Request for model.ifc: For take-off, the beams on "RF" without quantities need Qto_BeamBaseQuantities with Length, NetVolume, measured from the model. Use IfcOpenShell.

First a look at what the model holds.

```python
import ifcopenshell
import ifcopenshell.util.element
import ifcopenshell.util.unit

model = ifcopenshell.open("model.ifc")
print(model.schema)
for unit_type in ("LENGTHUNIT", "AREAUNIT", "VOLUMEUNIT"):
    print(unit_type, ifcopenshell.util.unit.calculate_unit_scale(model, unit_type))
storey = next(s for s in model.by_type("IfcBuildingStorey") if s.Name == "RF")
beams = [e for e in ifcopenshell.util.element.get_decomposition(storey) if e.is_a("IfcBeam")]
for e in sorted(beams, key=lambda e: e.id()):
    print(e.id(), e.is_a(), e.Name, list(ifcopenshell.util.element.get_psets(e, qtos_only=True)), sep=" | ")
```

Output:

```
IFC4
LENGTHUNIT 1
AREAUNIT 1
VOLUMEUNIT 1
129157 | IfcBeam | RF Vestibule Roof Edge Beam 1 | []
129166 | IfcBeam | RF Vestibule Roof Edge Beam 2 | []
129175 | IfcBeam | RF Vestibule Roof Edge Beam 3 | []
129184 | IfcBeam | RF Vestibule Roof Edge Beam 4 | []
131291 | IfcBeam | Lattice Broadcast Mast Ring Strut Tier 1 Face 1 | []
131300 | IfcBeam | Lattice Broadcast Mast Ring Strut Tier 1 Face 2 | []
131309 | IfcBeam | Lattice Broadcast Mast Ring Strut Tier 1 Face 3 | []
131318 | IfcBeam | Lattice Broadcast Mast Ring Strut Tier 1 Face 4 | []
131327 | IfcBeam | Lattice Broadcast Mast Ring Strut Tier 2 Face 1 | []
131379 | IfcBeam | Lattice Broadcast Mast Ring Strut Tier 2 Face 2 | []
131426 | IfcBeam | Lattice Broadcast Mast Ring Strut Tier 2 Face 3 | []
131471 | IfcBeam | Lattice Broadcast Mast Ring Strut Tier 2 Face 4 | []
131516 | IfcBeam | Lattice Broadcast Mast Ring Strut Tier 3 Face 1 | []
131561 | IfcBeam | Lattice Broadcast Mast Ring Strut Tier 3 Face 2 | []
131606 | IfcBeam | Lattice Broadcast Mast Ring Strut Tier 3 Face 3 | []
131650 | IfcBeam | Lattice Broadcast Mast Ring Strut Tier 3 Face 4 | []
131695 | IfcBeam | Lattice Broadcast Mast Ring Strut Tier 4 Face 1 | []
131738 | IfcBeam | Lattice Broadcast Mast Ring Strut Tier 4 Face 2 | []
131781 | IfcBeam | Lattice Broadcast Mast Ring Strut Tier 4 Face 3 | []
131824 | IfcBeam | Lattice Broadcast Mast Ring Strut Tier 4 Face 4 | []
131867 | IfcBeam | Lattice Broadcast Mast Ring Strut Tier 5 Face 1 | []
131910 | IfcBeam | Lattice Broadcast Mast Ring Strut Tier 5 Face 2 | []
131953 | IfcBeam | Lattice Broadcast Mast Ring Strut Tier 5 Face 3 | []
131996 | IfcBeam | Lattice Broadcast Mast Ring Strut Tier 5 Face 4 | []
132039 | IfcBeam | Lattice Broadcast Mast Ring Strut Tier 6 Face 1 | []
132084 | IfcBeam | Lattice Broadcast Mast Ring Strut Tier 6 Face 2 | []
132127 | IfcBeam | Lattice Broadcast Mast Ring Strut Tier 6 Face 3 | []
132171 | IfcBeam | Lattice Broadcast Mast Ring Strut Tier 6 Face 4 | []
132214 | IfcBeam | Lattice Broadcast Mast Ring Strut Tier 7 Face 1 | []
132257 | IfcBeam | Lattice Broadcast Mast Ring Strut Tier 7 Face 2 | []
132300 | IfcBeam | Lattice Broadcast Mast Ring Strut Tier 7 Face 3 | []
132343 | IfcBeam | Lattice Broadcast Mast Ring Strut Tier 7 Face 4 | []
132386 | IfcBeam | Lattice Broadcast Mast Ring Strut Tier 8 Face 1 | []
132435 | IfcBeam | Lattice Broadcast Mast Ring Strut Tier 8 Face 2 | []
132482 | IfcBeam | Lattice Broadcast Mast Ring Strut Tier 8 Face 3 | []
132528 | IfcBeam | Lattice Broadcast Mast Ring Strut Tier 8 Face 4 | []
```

```python
import ifcopenshell
import ifcopenshell.api.pset
import ifcopenshell.geom
import ifcopenshell.util.element
import ifcopenshell.util.shape
import ifcopenshell.util.unit

model = ifcopenshell.open("model.ifc")
unit_scale = ifcopenshell.util.unit.calculate_unit_scale(model)
volume_scale = ifcopenshell.util.unit.calculate_unit_scale(model, "VOLUMEUNIT")
settings = ifcopenshell.geom.settings()

storey = next(s for s in model.by_type("IfcBuildingStorey") if s.Name == "RF")
beams = [e for e in ifcopenshell.util.element.get_decomposition(storey) if e.is_a("IfcBeam")]

for e in sorted(beams, key=lambda e: e.id()):
    if ifcopenshell.util.element.get_psets(e, qtos_only=True, should_inherit=False):
        continue
    # Geometry comes back in metres, in the element's own axes.
    shape = ifcopenshell.geom.create_shape(settings, e)
    values = {
        "Length": ifcopenshell.util.shape.get_max_xyz(shape.geometry) / unit_scale,
        "NetVolume": ifcopenshell.util.shape.get_volume(shape.geometry) / volume_scale,
    }
    qto = ifcopenshell.api.pset.add_qto(model, product=e, name="Qto_BeamBaseQuantities")
    ifcopenshell.api.pset.edit_qto(model, qto=qto, properties=values)
    print(e.id(), {k: round(v, 3) for k, v in values.items()})

model.write("model_rev.ifc")
```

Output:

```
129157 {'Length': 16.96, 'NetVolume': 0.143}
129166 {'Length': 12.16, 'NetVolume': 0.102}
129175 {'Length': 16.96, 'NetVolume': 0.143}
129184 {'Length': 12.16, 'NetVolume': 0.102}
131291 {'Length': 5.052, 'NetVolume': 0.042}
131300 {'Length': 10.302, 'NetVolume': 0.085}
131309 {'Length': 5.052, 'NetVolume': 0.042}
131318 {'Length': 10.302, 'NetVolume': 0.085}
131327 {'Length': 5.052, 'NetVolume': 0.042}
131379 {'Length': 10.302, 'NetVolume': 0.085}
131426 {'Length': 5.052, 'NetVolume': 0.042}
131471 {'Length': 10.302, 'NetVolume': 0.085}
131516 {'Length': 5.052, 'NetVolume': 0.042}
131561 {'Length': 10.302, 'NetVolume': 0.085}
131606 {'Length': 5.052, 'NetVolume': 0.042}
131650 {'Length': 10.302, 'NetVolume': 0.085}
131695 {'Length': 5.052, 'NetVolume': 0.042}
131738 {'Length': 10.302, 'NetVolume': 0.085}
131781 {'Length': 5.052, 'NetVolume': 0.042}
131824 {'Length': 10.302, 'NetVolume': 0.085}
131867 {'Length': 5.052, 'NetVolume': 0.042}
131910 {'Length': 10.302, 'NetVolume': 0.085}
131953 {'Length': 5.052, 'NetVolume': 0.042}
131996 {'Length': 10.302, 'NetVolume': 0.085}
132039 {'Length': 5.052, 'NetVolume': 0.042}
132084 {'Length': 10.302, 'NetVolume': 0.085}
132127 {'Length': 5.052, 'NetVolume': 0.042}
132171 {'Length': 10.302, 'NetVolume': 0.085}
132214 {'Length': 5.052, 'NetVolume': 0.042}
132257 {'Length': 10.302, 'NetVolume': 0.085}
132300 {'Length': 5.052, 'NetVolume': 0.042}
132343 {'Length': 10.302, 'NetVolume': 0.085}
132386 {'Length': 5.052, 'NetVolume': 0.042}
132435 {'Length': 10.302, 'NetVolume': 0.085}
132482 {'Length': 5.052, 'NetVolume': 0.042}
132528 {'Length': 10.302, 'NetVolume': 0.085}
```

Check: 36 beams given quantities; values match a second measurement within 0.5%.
